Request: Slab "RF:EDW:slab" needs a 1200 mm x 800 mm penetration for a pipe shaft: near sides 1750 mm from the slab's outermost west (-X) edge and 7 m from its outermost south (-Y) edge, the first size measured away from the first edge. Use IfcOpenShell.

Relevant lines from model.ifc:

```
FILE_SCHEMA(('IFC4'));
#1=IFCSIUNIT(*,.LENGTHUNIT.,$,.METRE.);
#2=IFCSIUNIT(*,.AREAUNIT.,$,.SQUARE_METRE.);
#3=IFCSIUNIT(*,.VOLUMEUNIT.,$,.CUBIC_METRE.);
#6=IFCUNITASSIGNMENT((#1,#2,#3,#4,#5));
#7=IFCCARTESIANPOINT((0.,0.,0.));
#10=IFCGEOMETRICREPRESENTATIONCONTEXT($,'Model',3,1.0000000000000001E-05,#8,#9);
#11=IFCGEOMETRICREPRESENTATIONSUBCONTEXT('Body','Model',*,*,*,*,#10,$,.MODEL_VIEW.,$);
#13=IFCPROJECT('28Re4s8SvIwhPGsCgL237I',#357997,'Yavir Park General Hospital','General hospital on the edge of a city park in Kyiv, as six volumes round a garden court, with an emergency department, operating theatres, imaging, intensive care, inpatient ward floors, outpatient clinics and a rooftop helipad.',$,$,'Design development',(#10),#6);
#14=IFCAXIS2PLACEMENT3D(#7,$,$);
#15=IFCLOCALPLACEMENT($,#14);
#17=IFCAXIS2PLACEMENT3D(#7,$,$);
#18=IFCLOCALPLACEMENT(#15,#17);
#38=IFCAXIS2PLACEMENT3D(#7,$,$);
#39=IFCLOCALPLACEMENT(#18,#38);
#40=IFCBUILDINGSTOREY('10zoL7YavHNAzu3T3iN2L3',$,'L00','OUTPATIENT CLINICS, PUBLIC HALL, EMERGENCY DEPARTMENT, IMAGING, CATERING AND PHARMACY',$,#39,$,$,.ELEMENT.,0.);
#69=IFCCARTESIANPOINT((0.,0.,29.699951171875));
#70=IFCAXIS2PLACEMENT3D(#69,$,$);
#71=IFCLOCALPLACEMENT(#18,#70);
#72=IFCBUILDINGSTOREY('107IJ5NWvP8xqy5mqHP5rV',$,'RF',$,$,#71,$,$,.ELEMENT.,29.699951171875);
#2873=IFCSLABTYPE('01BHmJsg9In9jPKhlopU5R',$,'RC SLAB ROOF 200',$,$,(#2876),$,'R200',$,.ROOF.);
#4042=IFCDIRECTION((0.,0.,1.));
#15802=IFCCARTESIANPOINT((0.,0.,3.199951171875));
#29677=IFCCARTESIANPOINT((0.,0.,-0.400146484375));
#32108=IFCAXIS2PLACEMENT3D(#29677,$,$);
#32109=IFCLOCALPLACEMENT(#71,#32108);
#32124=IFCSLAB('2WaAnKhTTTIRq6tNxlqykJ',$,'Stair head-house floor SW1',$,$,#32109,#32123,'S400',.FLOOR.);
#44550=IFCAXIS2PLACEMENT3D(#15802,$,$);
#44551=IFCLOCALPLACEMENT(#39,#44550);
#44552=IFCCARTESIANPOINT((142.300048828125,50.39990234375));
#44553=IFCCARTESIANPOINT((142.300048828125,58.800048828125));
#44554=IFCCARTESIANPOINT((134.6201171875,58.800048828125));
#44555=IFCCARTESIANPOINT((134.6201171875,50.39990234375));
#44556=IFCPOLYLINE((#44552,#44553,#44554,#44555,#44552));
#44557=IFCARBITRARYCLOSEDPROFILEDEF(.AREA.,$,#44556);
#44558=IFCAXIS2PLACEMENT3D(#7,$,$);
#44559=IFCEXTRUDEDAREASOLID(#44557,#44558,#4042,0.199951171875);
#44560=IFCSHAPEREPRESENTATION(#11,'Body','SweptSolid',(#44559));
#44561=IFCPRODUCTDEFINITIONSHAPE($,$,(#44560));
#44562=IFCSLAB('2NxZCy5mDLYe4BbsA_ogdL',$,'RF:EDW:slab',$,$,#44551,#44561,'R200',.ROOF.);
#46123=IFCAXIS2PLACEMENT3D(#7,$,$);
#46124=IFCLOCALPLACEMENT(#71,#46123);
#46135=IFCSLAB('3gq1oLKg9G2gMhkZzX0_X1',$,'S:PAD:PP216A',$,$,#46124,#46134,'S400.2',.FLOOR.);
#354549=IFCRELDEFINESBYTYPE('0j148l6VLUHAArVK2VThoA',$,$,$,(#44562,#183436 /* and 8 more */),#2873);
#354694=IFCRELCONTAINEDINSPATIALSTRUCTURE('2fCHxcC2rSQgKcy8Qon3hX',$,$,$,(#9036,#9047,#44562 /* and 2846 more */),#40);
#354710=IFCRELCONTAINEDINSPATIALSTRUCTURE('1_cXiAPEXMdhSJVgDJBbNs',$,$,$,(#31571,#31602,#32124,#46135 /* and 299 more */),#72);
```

```python
import numpy as np
import ifcopenshell
import ifcopenshell.api.feature
import ifcopenshell.api.geometry
import ifcopenshell.api.root
import ifcopenshell.geom
import ifcopenshell.util.placement
import ifcopenshell.util.representation
import ifcopenshell.util.shape
import ifcopenshell.util.unit

model = ifcopenshell.open("model.ifc")
unit_scale = ifcopenshell.util.unit.calculate_unit_scale(model)
settings = ifcopenshell.geom.settings()


def volume(element):
    """Net volume in cubic metres, openings subtracted."""
    shape = ifcopenshell.geom.create_shape(settings, element)
    return ifcopenshell.util.shape.get_volume(shape.geometry)


slab = model.by_id(44562)
before = volume(slab)

# Extent in the slab's own axes, in metres. The edges named are its -X and -Y sides.
slab_shape = ifcopenshell.geom.create_shape(settings, slab)
vertices = ifcopenshell.util.shape.get_vertices(slab_shape.geometry)
x_min, y_min, bottom = vertices.min(axis=0)
top = vertices[:, 2].max()

opening = ifcopenshell.api.root.create_entity(model, ifc_class="IfcOpeningElement", name="Pipe shaft opening", predefined_type="OPENING")
context = ifcopenshell.util.representation.get_context(model, "Model", "Body", "MODEL_VIEW")
width, depth = 1.2, 0.8
outline = [(0.0, 0.0), (width, 0.0), (width, depth), (0.0, depth), (0.0, 0.0)]
# Overshoot both faces by 50 mm so the cut is clean.
shape = ifcopenshell.api.geometry.add_slab_representation(
    model, context=context, depth=top - bottom + 0.1, polyline=outline
)
ifcopenshell.api.geometry.assign_representation(model, product=opening, representation=shape)

matrix = ifcopenshell.util.placement.get_local_placement(slab.ObjectPlacement)
matrix[:, 3] = matrix @ np.append(np.array([x_min + 1.75, y_min + 7, bottom - 0.05]) / unit_scale, 1.0)
ifcopenshell.api.geometry.edit_object_placement(model, product=opening, matrix=matrix, is_si=False)
ifcopenshell.api.feature.add_feature(model, feature=opening, element=slab)

after = volume(slab)

print(f"slab volume {before:.3f} -> {after:.3f} m3")

model.write("model_rev.ifc")
```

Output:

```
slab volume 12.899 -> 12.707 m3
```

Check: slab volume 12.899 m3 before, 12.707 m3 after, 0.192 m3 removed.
